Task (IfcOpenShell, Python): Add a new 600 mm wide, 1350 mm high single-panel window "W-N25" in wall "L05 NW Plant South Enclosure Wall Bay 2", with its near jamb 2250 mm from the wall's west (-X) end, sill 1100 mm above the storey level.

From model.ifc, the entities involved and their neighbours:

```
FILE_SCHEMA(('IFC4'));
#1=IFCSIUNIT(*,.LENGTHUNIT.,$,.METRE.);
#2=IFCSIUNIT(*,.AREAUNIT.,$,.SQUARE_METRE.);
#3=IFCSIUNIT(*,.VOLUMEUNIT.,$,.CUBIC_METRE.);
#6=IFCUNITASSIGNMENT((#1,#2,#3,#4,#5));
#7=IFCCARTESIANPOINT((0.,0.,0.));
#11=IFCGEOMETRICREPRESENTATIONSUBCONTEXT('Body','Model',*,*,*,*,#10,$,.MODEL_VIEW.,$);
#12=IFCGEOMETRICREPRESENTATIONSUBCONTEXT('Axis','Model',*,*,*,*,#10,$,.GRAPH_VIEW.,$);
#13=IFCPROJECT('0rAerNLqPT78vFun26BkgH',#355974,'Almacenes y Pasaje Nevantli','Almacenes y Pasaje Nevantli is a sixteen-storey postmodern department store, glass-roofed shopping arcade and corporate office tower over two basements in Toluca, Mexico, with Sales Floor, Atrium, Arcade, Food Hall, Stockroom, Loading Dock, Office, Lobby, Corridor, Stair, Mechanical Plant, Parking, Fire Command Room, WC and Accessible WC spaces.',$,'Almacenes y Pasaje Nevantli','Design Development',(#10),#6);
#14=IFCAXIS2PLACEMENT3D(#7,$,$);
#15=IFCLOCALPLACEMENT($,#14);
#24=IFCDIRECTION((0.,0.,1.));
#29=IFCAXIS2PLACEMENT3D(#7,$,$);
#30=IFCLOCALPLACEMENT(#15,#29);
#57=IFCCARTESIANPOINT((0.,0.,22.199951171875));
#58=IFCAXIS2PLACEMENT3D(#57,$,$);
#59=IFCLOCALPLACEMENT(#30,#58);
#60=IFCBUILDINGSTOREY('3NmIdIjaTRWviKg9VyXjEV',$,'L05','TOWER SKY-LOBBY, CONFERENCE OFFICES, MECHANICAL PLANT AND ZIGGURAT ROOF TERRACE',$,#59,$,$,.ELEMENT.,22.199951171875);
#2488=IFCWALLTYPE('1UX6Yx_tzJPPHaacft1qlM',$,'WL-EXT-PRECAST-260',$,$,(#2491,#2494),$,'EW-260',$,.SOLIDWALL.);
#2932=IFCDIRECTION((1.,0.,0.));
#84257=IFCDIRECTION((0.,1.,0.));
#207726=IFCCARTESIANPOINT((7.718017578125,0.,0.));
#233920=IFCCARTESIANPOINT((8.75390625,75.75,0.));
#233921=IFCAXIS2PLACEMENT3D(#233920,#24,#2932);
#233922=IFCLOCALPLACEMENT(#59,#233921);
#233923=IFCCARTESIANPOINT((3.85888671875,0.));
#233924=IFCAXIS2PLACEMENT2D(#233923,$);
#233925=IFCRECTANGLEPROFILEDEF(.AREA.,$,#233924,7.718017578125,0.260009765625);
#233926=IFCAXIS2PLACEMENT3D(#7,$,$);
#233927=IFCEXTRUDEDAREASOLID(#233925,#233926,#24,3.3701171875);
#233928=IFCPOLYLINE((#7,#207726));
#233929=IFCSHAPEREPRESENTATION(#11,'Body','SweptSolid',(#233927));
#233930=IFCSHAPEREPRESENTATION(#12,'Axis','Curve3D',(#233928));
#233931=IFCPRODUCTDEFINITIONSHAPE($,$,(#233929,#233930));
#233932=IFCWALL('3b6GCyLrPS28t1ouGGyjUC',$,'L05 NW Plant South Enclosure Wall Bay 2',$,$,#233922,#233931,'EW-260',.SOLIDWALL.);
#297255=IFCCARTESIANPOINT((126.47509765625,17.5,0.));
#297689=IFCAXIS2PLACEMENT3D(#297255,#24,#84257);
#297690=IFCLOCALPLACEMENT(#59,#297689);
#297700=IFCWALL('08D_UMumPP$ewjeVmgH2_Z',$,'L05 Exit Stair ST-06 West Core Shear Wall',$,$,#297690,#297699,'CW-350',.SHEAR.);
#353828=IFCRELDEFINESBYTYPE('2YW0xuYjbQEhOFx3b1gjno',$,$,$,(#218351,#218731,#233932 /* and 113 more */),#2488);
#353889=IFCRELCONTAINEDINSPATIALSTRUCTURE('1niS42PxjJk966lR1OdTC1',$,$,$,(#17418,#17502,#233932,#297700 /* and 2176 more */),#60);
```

```python
import numpy as np
import ifcopenshell
import ifcopenshell.api.feature
import ifcopenshell.api.geometry
import ifcopenshell.api.root
import ifcopenshell.api.spatial
import ifcopenshell.geom
import ifcopenshell.util.element
import ifcopenshell.util.placement
import ifcopenshell.util.representation
import ifcopenshell.util.shape
import ifcopenshell.util.unit

model = ifcopenshell.open("model.ifc")
unit_scale = ifcopenshell.util.unit.calculate_unit_scale(model)
settings = ifcopenshell.geom.settings()


def volume(element):
    """Net volume in cubic metres, openings subtracted."""
    shape = ifcopenshell.geom.create_shape(settings, element)
    return ifcopenshell.util.shape.get_volume(shape.geometry)


wall = model.by_id(233932)
storey = ifcopenshell.util.element.get_container(wall, ifc_class="IfcBuildingStorey")
context = ifcopenshell.util.representation.get_context(model, "Model", "Body", "MODEL_VIEW")
before = volume(wall)

width, height, from_end, sill = 0.6, 1.35, 2.25, 1.1  # metres

# The wall runs along its own X axis, and the end named is its -X end.
wall_shape = ifcopenshell.geom.create_shape(settings, wall)
x, y, z = ifcopenshell.util.shape.get_vertices(wall_shape.geometry).T
start = x.min() + from_end
face, thickness = float(y.min()), float(y.max() - y.min())
wall_matrix = ifcopenshell.util.placement.get_local_placement(wall.ObjectPlacement)
level = ifcopenshell.util.placement.get_local_placement(storey.ObjectPlacement)[2, 3]


def in_wall(x, y):
    """Placement at x, y metres in the wall's axes, at sill height."""
    matrix = wall_matrix.copy()
    matrix[:, 3] = wall_matrix @ np.array([x / unit_scale, y / unit_scale, 0.0, 1.0])
    matrix[2, 3] = level + sill / unit_scale
    return matrix


# Opening: a box that overshoots both wall faces by 50 mm.
opening = ifcopenshell.api.root.create_entity(model, ifc_class="IfcOpeningElement", predefined_type="OPENING")
box = ifcopenshell.api.geometry.add_wall_representation(
    model, context=context, length=width, height=height, thickness=thickness + 0.1
)
ifcopenshell.api.geometry.assign_representation(model, product=opening, representation=box)
ifcopenshell.api.geometry.edit_object_placement(model, product=opening, matrix=in_wall(start, face - 0.05), is_si=False)
ifcopenshell.api.feature.add_feature(model, feature=opening, element=wall)

window = ifcopenshell.api.root.create_entity(model, ifc_class="IfcWindow", name="W-N25", predefined_type="WINDOW")
window.OverallWidth, window.OverallHeight = width / unit_scale, height / unit_scale
window.PartitioningType = "SINGLE_PANEL"
body = ifcopenshell.api.geometry.add_window_representation(
    model,
    context=context,
    overall_width=window.OverallWidth,
    overall_height=window.OverallHeight,
    partition_type="SINGLE_PANEL",
)
ifcopenshell.api.geometry.assign_representation(model, product=window, representation=body)
ifcopenshell.api.spatial.assign_container(model, products=[window], relating_structure=storey)
ifcopenshell.api.feature.add_filling(model, opening=opening, element=window)

# Centre the window in the wall's thickness.
ifcopenshell.api.geometry.edit_object_placement(model, product=window, matrix=in_wall(start, face), is_si=False)
window_shape = ifcopenshell.geom.create_shape(settings, window)
depth = ifcopenshell.util.shape.get_vertices(window_shape.geometry)[:, 1]
offset = face + thickness / 2 - (depth.min() + depth.max()) / 2
ifcopenshell.api.geometry.edit_object_placement(model, product=window, matrix=in_wall(start, offset), is_si=False)

after = volume(wall)

print(f"wall volume {before:.3f} -> {after:.3f} m3")

model.write("model_rev.ifc")
```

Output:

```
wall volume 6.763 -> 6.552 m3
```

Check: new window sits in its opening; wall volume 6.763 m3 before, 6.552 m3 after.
